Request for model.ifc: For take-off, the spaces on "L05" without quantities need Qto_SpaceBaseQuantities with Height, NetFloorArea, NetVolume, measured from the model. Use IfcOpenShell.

First a look at what the model holds.

```python
import ifcopenshell
import ifcopenshell.util.element
import ifcopenshell.util.unit

model = ifcopenshell.open("model.ifc")
print(model.schema)
for unit_type in ("LENGTHUNIT", "AREAUNIT", "VOLUMEUNIT"):
    print(unit_type, ifcopenshell.util.unit.calculate_unit_scale(model, unit_type))
storey = next(s for s in model.by_type("IfcBuildingStorey") if s.Name == "L05")
spaces = [e for e in ifcopenshell.util.element.get_decomposition(storey) if e.is_a("IfcSpace")]
for e in sorted(spaces, key=lambda e: e.id()):
    print(e.id(), e.is_a(), e.Name, list(ifcopenshell.util.element.get_psets(e, qtos_only=True)), sep=" | ")
```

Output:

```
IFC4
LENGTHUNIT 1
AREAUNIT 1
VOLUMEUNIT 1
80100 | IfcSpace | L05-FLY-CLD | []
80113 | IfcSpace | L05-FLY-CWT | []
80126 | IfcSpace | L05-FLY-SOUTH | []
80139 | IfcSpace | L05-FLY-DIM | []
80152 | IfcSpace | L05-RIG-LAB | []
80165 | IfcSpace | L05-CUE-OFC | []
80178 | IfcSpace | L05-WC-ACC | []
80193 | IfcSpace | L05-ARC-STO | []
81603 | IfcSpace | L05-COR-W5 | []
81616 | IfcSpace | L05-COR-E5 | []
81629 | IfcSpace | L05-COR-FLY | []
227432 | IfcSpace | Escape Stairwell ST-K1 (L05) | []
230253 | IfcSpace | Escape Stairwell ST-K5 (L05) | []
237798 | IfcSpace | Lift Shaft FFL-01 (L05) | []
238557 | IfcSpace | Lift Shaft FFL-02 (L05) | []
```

```python
import ifcopenshell
import ifcopenshell.api.pset
import ifcopenshell.geom
import ifcopenshell.util.element
import ifcopenshell.util.shape
import ifcopenshell.util.unit

model = ifcopenshell.open("model.ifc")
unit_scale = ifcopenshell.util.unit.calculate_unit_scale(model)
area_scale = ifcopenshell.util.unit.calculate_unit_scale(model, "AREAUNIT")
volume_scale = ifcopenshell.util.unit.calculate_unit_scale(model, "VOLUMEUNIT")
settings = ifcopenshell.geom.settings()

storey = next(s for s in model.by_type("IfcBuildingStorey") if s.Name == "L05")
spaces = [e for e in ifcopenshell.util.element.get_decomposition(storey) if e.is_a("IfcSpace")]

for e in sorted(spaces, key=lambda e: e.id()):
    if ifcopenshell.util.element.get_psets(e, qtos_only=True, should_inherit=False):
        continue
    # Geometry comes back in metres, in the element's own axes.
    shape = ifcopenshell.geom.create_shape(settings, e)
    values = {
        "Height": ifcopenshell.util.shape.get_z(shape.geometry) / unit_scale,
        "NetFloorArea": ifcopenshell.util.shape.get_footprint_area(shape.geometry) / area_scale,
        "NetVolume": ifcopenshell.util.shape.get_volume(shape.geometry) / volume_scale,
    }
    qto = ifcopenshell.api.pset.add_qto(model, product=e, name="Qto_SpaceBaseQuantities")
    ifcopenshell.api.pset.edit_qto(model, qto=qto, properties=values)
    print(e.id(), {k: round(v, 3) for k, v in values.items()})

model.write("model_rev.ifc")
```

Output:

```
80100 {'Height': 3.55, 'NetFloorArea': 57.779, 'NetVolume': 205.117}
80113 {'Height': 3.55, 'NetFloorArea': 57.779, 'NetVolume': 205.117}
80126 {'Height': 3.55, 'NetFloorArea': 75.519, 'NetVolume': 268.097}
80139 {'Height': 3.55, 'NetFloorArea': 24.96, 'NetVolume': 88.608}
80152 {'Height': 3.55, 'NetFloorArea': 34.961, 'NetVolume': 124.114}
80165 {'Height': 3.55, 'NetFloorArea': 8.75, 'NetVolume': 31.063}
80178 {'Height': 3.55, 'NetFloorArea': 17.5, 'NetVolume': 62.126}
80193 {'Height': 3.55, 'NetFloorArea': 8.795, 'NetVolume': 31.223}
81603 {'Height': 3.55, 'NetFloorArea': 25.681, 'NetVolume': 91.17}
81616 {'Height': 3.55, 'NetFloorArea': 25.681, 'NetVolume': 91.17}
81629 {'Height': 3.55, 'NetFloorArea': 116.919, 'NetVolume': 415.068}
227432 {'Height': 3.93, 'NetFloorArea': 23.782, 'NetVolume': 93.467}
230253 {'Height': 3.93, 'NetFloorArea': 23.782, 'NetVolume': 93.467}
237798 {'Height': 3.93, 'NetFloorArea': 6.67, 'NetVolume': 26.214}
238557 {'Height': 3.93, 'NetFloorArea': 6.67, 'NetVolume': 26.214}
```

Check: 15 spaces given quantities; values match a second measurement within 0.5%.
